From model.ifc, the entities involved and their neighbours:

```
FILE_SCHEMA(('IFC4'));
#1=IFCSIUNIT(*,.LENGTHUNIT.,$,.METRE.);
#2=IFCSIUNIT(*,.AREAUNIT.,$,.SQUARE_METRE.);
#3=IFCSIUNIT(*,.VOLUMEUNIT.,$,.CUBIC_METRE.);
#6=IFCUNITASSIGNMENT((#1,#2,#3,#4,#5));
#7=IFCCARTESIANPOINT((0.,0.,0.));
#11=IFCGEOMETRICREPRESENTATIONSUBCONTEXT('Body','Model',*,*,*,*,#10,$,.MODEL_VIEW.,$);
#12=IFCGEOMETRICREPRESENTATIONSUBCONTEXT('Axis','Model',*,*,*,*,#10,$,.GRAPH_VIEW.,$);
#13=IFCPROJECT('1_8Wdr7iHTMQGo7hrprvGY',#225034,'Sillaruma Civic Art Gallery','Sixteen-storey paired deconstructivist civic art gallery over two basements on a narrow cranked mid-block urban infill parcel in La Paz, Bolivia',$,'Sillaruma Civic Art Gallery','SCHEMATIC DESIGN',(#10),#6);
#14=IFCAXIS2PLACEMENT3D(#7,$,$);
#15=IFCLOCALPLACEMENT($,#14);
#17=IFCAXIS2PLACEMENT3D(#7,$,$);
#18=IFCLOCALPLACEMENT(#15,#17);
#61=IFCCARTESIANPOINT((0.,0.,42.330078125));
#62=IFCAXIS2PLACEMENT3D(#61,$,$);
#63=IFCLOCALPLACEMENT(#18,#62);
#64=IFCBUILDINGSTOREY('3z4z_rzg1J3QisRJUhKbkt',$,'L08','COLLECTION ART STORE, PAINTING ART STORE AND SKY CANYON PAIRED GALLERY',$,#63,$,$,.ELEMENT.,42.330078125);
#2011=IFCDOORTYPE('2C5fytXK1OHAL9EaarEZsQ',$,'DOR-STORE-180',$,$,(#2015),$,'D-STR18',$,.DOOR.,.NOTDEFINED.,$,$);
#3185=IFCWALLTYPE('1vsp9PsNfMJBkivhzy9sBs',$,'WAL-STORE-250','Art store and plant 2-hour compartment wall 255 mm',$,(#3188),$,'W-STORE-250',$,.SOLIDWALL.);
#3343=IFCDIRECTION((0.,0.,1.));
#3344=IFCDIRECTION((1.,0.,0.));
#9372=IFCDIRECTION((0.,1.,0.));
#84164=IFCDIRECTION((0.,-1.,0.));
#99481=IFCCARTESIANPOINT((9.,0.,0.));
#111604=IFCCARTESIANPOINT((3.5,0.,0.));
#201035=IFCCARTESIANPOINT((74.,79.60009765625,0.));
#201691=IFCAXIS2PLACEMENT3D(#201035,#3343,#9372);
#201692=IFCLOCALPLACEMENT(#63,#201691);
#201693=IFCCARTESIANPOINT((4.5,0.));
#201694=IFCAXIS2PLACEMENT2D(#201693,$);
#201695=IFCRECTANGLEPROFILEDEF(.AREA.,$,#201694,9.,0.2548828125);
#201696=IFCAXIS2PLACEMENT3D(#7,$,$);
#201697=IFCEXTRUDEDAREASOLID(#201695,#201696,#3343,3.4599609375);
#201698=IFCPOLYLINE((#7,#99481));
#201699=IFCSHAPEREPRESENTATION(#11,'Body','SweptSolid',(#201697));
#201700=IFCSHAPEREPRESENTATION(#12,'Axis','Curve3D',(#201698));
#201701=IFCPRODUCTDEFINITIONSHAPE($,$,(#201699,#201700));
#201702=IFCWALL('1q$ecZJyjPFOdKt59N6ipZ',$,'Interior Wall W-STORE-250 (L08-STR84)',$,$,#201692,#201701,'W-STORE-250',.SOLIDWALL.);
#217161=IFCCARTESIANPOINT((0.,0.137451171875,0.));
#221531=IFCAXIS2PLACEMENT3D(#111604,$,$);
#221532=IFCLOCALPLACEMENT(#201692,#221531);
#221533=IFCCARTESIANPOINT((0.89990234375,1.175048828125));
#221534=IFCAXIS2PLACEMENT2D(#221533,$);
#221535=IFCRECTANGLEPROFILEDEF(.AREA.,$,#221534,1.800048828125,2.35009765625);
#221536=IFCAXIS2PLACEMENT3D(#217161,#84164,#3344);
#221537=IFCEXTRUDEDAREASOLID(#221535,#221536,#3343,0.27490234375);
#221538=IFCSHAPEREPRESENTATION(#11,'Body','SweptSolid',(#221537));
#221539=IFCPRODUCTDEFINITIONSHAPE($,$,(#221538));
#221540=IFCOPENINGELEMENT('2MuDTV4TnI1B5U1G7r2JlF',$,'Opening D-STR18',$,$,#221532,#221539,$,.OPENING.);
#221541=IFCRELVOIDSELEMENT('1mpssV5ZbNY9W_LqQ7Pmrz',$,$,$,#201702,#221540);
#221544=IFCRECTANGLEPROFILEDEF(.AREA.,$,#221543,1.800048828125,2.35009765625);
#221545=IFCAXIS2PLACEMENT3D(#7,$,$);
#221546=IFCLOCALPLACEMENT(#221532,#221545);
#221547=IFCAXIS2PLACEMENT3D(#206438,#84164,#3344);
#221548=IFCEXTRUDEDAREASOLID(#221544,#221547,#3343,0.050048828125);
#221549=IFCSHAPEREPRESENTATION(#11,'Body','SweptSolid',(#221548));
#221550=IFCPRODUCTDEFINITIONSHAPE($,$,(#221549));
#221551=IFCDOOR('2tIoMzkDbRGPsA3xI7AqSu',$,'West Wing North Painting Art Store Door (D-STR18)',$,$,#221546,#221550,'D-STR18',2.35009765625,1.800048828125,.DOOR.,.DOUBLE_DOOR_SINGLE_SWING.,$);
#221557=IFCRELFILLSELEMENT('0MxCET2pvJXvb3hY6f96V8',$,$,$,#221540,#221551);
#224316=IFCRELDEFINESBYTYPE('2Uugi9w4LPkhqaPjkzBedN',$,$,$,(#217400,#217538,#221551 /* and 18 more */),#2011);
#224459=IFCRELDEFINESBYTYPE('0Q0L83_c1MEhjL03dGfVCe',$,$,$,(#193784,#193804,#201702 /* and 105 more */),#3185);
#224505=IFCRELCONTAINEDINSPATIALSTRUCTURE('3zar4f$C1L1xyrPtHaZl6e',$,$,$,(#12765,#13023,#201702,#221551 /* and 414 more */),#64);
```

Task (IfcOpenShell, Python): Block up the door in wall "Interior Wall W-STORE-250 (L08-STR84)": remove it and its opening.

```python
import ifcopenshell
import ifcopenshell.api.feature
import ifcopenshell.api.root
import ifcopenshell.geom
import ifcopenshell.util.shape

model = ifcopenshell.open("model.ifc")
settings = ifcopenshell.geom.settings()


def volume(element):
    """Net volume in cubic metres, openings subtracted."""
    shape = ifcopenshell.geom.create_shape(settings, element)
    return ifcopenshell.util.shape.get_volume(shape.geometry)


door = model.by_id(221551)
opening = door.FillsVoids[0].RelatingOpeningElement
wall = opening.VoidsElements[0].RelatingBuildingElement
before = volume(wall)

ifcopenshell.api.root.remove_product(model, product=door)
ifcopenshell.api.feature.remove_feature(model, feature=opening)

after = volume(wall)

print(f"wall volume {before:.3f} -> {after:.3f} m3")

model.write("model_rev.ifc")
```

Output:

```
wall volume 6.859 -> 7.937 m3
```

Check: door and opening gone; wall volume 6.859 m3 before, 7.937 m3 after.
